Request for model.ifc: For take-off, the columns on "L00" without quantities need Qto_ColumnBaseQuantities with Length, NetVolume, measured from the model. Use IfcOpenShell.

First a look at what the model holds.

```python
import ifcopenshell
import ifcopenshell.util.element
import ifcopenshell.util.unit

model = ifcopenshell.open("model.ifc")
print(model.schema)
for unit_type in ("LENGTHUNIT", "AREAUNIT", "VOLUMEUNIT"):
    print(unit_type, ifcopenshell.util.unit.calculate_unit_scale(model, unit_type))
storey = next(s for s in model.by_type("IfcBuildingStorey") if s.Name == "L00")
columns = [e for e in ifcopenshell.util.element.get_decomposition(storey) if e.is_a("IfcColumn")]
for e in sorted(columns, key=lambda e: e.id()):
    print(e.id(), e.is_a(), e.Name, list(ifcopenshell.util.element.get_psets(e, qtos_only=True)), sep=" | ")
```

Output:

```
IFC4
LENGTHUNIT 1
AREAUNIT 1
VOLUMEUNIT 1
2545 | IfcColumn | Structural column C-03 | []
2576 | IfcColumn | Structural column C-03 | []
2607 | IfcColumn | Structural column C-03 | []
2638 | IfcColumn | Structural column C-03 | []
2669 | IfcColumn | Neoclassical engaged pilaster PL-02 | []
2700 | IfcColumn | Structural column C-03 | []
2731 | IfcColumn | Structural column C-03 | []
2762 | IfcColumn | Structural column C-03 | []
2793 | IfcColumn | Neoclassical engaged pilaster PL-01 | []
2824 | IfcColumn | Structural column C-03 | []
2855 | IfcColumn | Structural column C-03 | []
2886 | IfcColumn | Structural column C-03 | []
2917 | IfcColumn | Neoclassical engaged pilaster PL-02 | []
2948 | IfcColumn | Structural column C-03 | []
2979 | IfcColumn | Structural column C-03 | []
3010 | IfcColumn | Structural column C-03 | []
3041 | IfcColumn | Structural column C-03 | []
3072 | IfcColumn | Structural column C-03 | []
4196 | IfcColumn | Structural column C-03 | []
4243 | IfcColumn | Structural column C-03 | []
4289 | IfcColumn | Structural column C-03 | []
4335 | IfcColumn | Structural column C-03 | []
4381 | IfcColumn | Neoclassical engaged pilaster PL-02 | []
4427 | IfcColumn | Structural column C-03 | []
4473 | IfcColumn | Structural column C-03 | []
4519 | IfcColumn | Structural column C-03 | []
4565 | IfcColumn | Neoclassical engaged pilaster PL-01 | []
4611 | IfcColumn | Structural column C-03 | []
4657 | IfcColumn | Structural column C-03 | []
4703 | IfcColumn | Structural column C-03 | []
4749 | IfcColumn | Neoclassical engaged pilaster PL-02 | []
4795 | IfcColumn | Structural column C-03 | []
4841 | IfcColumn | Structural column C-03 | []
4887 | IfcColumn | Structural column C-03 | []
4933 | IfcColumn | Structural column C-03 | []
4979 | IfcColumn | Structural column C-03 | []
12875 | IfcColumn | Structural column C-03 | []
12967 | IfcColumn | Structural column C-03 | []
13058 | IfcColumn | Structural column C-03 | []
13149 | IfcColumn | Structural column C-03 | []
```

```python
import ifcopenshell
import ifcopenshell.api.pset
import ifcopenshell.geom
import ifcopenshell.util.element
import ifcopenshell.util.shape
import ifcopenshell.util.unit

model = ifcopenshell.open("model.ifc")
unit_scale = ifcopenshell.util.unit.calculate_unit_scale(model)
volume_scale = ifcopenshell.util.unit.calculate_unit_scale(model, "VOLUMEUNIT")
settings = ifcopenshell.geom.settings()

storey = next(s for s in model.by_type("IfcBuildingStorey") if s.Name == "L00")
columns = [e for e in ifcopenshell.util.element.get_decomposition(storey) if e.is_a("IfcColumn")]

for e in sorted(columns, key=lambda e: e.id()):
    if ifcopenshell.util.element.get_psets(e, qtos_only=True, should_inherit=False):
        continue
    # Geometry comes back in metres, in the element's own axes.
    shape = ifcopenshell.geom.create_shape(settings, e)
    values = {
        "Length": ifcopenshell.util.shape.get_z(shape.geometry) / unit_scale,
        "NetVolume": ifcopenshell.util.shape.get_volume(shape.geometry) / volume_scale,
    }
    qto = ifcopenshell.api.pset.add_qto(model, product=e, name="Qto_ColumnBaseQuantities")
    ifcopenshell.api.pset.edit_qto(model, qto=qto, properties=values)
    print(e.id(), {k: round(v, 3) for k, v in values.items()})

model.write("model_v2.ifc")
```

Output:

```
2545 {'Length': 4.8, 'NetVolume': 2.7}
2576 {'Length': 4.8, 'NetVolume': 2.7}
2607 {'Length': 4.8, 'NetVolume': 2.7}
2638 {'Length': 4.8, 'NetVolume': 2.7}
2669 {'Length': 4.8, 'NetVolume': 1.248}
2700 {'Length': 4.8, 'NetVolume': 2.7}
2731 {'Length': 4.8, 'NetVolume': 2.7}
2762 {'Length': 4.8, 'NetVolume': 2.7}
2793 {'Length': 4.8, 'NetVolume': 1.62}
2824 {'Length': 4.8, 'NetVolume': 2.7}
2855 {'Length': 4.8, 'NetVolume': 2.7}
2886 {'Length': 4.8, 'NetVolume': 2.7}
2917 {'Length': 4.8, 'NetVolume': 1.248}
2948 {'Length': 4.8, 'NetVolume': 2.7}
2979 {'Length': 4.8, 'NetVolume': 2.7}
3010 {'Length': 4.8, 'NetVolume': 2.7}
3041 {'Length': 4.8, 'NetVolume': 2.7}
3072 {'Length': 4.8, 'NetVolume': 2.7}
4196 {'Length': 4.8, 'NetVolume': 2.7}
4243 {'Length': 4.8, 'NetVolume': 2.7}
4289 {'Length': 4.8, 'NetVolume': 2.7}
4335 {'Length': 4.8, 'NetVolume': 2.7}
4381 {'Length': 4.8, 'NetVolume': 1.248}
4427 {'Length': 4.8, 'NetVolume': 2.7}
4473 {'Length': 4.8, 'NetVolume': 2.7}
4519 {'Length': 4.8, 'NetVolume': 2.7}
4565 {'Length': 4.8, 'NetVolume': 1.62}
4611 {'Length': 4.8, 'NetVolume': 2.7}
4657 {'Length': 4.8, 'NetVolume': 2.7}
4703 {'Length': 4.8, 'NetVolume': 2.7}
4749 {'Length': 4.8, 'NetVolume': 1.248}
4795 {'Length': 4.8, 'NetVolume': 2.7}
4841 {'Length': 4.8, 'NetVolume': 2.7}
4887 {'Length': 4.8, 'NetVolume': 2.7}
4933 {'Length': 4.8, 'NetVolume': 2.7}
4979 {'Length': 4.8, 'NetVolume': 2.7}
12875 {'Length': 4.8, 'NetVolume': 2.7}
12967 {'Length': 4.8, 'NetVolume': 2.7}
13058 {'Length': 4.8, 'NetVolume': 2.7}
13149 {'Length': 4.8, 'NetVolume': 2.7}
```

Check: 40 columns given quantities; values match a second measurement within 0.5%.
